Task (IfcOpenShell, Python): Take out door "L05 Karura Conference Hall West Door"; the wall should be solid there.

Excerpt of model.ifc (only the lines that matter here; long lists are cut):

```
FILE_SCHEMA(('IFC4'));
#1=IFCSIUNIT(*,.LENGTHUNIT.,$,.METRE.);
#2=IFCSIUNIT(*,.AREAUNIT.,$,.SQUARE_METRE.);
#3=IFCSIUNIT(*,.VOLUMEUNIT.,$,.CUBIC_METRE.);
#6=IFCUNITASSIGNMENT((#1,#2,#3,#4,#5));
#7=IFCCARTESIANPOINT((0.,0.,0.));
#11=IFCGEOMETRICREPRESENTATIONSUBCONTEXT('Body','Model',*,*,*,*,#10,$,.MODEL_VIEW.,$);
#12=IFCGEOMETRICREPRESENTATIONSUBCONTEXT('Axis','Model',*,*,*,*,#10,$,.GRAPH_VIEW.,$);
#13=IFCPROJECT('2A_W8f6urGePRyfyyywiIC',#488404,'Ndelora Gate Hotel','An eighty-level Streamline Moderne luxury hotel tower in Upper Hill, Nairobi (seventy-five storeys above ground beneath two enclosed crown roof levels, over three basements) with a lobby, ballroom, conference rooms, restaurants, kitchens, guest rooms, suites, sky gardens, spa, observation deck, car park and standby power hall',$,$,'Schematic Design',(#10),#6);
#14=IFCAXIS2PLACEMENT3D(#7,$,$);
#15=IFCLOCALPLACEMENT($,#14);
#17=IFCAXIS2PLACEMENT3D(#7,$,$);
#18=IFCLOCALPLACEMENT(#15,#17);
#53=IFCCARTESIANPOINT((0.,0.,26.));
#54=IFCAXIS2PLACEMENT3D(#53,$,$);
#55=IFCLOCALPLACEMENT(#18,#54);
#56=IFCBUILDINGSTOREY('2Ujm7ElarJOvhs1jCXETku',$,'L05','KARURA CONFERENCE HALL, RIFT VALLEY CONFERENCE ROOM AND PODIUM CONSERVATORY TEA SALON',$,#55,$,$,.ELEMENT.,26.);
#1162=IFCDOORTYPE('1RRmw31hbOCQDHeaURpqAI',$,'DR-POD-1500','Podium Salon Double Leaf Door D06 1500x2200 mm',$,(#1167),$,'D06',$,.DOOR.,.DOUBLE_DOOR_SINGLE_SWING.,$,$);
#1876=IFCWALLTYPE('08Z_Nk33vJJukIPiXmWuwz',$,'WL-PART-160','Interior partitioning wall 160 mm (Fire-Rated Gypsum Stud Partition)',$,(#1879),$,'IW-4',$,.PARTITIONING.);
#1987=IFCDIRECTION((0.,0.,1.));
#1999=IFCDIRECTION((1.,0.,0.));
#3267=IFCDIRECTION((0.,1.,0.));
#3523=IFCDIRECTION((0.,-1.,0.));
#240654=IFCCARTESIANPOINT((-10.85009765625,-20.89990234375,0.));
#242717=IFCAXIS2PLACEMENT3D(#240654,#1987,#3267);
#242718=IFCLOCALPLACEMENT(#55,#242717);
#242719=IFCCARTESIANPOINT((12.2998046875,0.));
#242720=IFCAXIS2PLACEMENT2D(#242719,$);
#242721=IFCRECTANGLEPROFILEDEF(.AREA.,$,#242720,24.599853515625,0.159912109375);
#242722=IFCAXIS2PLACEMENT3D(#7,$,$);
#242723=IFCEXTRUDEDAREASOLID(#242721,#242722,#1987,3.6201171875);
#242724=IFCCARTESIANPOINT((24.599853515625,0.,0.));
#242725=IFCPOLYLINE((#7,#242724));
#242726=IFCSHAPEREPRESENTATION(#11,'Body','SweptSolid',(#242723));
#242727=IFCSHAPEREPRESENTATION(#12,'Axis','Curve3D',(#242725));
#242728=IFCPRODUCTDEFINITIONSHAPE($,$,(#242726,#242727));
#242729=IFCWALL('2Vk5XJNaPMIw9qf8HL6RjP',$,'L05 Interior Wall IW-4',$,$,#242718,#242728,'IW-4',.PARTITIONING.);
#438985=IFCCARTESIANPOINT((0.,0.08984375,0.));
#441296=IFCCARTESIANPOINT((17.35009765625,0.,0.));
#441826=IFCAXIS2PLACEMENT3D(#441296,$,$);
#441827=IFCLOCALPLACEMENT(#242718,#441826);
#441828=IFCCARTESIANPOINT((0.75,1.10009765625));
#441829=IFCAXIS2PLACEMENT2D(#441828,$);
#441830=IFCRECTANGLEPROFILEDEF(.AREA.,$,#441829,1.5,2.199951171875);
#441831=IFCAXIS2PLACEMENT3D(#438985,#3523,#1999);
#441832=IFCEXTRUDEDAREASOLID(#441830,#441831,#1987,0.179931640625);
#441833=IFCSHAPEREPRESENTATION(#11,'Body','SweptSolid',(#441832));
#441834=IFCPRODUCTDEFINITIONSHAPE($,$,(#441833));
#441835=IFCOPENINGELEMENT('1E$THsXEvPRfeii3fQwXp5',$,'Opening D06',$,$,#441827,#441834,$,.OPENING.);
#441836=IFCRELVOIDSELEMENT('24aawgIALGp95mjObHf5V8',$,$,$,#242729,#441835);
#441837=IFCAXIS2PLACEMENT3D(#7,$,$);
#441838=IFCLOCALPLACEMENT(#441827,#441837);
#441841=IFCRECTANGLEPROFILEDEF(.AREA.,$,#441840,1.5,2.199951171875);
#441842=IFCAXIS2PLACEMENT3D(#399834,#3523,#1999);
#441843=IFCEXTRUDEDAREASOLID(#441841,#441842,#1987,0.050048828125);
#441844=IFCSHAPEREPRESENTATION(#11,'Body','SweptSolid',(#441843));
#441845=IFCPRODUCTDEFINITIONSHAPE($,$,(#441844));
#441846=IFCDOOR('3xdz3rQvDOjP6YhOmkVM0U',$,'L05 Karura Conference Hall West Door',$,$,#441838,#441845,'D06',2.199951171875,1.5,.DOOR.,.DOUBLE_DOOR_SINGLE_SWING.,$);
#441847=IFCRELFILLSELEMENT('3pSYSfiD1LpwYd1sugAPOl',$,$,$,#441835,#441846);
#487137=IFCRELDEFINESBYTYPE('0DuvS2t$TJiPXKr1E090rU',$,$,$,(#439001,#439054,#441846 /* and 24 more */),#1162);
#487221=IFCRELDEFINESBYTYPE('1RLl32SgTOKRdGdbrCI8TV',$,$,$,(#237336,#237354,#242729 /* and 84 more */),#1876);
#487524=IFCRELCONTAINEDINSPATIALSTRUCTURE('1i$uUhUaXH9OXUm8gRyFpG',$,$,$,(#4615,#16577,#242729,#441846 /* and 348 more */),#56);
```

```python
import ifcopenshell
import ifcopenshell.api.feature
import ifcopenshell.api.root
import ifcopenshell.geom
import ifcopenshell.util.shape

model = ifcopenshell.open("model.ifc")
settings = ifcopenshell.geom.settings()


def volume(element):
    """Net volume in cubic metres, openings subtracted."""
    shape = ifcopenshell.geom.create_shape(settings, element)
    return ifcopenshell.util.shape.get_volume(shape.geometry)


door = model.by_id(441846)
opening = door.FillsVoids[0].RelatingOpeningElement
wall = opening.VoidsElements[0].RelatingBuildingElement
before = volume(wall)

ifcopenshell.api.root.remove_product(model, product=door)
ifcopenshell.api.feature.remove_feature(model, feature=opening)

after = volume(wall)

print(f"wall volume {before:.3f} -> {after:.3f} m3")

model.write("model_v2.ifc")
```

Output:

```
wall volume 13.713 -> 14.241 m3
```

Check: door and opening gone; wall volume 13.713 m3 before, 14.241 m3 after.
